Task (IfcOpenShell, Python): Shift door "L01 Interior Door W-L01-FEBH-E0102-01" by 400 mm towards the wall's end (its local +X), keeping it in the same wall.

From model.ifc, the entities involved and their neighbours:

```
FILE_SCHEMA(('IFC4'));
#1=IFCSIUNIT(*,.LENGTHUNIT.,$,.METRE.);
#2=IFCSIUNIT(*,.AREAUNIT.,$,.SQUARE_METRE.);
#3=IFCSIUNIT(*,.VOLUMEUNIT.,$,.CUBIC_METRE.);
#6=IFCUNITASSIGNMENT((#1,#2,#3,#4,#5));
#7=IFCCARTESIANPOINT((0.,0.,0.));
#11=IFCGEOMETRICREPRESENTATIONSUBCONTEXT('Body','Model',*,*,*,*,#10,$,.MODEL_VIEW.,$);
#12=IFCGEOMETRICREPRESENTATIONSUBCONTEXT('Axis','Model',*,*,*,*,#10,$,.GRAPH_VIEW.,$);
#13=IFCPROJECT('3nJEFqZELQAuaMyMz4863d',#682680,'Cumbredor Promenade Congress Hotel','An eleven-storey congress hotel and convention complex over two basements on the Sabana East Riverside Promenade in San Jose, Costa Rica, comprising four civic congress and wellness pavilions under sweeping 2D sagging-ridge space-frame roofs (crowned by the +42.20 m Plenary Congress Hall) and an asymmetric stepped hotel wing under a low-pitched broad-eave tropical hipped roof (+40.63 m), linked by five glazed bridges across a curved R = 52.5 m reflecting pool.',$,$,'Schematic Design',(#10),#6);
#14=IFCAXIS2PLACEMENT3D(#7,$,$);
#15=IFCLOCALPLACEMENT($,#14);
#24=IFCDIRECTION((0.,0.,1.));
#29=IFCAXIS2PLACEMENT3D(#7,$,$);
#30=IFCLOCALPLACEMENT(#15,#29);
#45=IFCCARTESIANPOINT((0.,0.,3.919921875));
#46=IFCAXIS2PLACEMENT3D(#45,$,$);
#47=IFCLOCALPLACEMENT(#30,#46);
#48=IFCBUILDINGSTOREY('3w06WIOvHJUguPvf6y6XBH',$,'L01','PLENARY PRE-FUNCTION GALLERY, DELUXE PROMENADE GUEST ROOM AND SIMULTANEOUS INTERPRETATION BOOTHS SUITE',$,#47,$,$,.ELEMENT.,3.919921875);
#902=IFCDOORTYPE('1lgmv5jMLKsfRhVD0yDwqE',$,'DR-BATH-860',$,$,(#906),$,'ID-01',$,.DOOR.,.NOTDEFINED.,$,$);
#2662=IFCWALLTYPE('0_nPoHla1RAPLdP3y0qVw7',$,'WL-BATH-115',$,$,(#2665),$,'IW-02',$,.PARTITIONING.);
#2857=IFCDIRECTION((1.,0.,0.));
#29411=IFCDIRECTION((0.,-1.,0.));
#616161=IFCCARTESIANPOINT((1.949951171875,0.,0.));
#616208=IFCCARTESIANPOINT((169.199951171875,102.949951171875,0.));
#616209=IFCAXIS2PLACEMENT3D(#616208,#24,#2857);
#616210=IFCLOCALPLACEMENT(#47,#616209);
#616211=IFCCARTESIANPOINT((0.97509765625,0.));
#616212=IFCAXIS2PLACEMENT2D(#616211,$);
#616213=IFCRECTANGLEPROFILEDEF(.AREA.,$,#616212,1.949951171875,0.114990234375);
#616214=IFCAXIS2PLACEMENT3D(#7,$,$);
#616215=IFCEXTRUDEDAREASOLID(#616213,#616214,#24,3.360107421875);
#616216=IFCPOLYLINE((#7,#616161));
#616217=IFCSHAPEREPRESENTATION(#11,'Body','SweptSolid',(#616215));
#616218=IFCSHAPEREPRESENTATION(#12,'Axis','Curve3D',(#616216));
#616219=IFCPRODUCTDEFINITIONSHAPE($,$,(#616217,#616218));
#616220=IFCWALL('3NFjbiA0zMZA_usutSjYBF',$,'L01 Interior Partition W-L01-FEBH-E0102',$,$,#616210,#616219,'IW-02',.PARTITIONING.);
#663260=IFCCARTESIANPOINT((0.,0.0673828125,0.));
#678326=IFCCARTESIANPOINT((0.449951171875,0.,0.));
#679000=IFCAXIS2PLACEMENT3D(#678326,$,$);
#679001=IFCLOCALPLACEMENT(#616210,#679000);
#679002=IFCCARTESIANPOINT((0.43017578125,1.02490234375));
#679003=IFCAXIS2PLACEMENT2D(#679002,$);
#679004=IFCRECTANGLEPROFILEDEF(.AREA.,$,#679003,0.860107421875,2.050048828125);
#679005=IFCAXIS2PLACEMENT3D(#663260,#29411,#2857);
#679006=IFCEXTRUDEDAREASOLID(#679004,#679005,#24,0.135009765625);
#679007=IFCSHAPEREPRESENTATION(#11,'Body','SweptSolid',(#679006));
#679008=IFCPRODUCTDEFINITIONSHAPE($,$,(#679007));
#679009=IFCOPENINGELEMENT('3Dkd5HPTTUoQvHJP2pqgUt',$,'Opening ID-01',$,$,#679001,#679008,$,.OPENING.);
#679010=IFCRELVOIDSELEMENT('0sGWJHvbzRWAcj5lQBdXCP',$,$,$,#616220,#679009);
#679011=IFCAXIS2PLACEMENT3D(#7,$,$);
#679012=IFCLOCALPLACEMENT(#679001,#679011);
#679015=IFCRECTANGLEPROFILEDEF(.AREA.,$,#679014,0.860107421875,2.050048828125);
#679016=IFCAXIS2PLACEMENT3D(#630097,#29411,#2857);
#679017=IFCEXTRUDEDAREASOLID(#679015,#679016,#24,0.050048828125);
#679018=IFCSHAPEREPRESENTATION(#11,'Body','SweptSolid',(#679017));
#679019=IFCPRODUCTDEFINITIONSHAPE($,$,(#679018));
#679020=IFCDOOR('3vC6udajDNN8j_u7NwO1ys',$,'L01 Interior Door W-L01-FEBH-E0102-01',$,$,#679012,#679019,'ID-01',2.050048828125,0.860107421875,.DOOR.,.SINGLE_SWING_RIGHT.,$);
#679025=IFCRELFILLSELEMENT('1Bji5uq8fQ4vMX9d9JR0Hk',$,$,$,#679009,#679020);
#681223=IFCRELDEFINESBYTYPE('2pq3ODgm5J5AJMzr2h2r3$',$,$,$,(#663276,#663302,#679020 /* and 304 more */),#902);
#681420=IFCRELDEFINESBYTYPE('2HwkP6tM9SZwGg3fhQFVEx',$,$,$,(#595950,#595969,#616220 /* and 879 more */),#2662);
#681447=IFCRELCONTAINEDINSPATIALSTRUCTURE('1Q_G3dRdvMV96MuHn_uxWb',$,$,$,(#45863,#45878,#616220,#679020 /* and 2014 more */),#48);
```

```python
import ifcopenshell
import ifcopenshell.api.geometry
import ifcopenshell.util.placement

model = ifcopenshell.open("model.ifc")

door = model.by_guid("3vC6udajDNN8j_u7NwO1ys")
opening = door.FillsVoids[0].RelatingOpeningElement
wall = opening.VoidsElements[0].RelatingBuildingElement

wall_matrix = ifcopenshell.util.placement.get_local_placement(wall.ObjectPlacement)
shift = wall_matrix[:3, 0] * 0.4
before = ifcopenshell.util.placement.get_local_placement(door.ObjectPlacement)[:3, 3].copy()

# The door is placed relative to its opening, so it follows when the opening moves.
matrix = ifcopenshell.util.placement.get_local_placement(opening.ObjectPlacement)
matrix[:3, 3] += shift
ifcopenshell.api.geometry.edit_object_placement(
    model, product=opening, matrix=matrix, is_si=False, should_transform_children=True
)

after = ifcopenshell.util.placement.get_local_placement(door.ObjectPlacement)[:3, 3]
print("door moved by", (after - before).round(3) + 0.0)

model.write("model-out.ifc")
```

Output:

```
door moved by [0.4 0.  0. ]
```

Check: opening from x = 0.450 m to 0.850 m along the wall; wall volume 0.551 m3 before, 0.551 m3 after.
